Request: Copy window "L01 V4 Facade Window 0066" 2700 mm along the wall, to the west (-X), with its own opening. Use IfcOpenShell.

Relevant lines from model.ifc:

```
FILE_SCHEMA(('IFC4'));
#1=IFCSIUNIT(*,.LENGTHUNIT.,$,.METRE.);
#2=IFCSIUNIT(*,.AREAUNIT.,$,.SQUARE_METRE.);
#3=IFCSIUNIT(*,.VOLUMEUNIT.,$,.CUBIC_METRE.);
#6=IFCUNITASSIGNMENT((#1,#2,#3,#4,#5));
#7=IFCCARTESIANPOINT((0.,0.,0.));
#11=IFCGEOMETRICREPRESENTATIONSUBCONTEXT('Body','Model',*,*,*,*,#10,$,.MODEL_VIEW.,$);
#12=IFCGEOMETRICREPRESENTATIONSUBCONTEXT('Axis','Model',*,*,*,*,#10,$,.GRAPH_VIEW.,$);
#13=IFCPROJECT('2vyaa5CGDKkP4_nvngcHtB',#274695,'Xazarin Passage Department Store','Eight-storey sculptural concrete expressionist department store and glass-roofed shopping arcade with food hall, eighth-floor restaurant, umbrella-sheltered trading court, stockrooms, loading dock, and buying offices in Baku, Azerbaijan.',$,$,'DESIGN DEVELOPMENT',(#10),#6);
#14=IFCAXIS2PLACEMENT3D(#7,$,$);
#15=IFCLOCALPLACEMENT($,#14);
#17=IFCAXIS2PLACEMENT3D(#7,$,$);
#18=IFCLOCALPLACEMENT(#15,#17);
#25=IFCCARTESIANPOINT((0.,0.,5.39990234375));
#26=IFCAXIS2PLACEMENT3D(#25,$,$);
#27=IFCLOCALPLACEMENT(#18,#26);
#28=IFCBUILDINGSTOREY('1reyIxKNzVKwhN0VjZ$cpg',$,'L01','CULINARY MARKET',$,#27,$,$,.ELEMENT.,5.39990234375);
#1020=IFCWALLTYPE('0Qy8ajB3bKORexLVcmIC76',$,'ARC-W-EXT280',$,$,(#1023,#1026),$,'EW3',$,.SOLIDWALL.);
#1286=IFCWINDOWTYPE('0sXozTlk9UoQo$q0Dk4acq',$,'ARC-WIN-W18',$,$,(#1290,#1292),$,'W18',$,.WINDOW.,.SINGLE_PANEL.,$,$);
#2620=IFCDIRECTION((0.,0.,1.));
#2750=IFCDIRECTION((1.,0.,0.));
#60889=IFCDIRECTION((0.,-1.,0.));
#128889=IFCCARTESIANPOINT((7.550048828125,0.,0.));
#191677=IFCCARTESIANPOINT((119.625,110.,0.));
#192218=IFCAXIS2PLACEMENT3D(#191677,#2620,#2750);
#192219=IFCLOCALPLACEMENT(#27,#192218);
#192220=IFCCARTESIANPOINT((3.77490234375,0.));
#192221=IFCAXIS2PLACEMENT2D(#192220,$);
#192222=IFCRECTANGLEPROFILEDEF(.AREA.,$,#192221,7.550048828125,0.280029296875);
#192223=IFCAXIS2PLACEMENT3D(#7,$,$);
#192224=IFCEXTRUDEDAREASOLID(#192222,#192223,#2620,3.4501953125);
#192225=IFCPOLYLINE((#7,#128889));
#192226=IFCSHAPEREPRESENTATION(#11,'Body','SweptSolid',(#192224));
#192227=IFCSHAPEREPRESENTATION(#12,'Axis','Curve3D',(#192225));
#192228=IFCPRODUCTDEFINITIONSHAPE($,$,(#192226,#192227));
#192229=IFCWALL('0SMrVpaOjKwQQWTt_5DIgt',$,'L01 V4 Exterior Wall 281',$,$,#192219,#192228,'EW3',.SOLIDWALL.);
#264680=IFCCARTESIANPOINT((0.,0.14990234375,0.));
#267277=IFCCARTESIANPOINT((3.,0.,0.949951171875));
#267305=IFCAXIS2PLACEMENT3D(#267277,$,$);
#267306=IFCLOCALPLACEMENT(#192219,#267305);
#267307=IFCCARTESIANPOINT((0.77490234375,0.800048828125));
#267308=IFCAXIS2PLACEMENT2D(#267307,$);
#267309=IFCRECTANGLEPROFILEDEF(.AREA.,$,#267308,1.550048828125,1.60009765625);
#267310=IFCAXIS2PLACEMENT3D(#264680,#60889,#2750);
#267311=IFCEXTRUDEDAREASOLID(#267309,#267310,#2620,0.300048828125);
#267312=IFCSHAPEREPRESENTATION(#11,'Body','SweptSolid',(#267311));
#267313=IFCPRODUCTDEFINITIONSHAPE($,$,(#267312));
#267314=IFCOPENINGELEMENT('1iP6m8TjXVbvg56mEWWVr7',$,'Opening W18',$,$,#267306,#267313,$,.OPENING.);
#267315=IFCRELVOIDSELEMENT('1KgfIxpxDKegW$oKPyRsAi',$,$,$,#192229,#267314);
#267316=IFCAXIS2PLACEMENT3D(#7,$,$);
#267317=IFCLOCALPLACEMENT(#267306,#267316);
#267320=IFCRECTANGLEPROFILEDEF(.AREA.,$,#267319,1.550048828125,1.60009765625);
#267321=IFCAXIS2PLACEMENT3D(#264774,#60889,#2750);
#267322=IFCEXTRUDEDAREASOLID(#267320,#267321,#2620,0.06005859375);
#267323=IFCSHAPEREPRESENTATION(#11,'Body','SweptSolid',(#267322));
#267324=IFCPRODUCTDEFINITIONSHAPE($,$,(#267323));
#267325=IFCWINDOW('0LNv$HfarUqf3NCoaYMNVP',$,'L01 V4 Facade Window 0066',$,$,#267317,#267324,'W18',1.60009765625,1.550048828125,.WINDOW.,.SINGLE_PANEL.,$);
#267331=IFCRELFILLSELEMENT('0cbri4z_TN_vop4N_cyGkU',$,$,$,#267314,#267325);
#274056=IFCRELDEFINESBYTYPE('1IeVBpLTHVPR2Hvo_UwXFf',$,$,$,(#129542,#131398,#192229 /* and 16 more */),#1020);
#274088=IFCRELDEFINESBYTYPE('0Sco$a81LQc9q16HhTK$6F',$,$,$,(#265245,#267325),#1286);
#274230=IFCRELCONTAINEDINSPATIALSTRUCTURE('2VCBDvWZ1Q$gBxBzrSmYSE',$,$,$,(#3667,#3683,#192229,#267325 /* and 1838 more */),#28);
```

```python
import ifcopenshell
import ifcopenshell.api.feature
import ifcopenshell.api.geometry
import ifcopenshell.api.root
import ifcopenshell.geom
import ifcopenshell.util.element
import ifcopenshell.util.placement
import ifcopenshell.util.shape

model = ifcopenshell.open("model.ifc")
settings = ifcopenshell.geom.settings()


def volume(element):
    """Net volume in cubic metres, openings subtracted."""
    shape = ifcopenshell.geom.create_shape(settings, element)
    return ifcopenshell.util.shape.get_volume(shape.geometry)


window = model.by_id(267325)
opening = window.FillsVoids[0].RelatingOpeningElement
wall = opening.VoidsElements[0].RelatingBuildingElement
before = volume(wall)
shift = ifcopenshell.util.placement.get_local_placement(wall.ObjectPlacement)[:3, 0] * -2.7

# copy_class copies the void relationship, type, container and properties, but no geometry.
new_opening = ifcopenshell.api.root.copy_class(model, product=opening)
new_opening.Representation = ifcopenshell.util.element.copy_deep(
    model, opening.Representation, exclude=["IfcGeometricRepresentationContext", "IfcRepresentationMap"]
)
new_window = ifcopenshell.api.root.copy_class(model, product=window)
new_window.Representation = ifcopenshell.util.element.copy_deep(
    model, window.Representation, exclude=["IfcGeometricRepresentationContext", "IfcRepresentationMap"]
)
new_window.Tag = None
ifcopenshell.api.feature.add_filling(model, opening=new_opening, element=new_window)

for old, new in ((opening, new_opening), (window, new_window)):
    matrix = ifcopenshell.util.placement.get_local_placement(old.ObjectPlacement)
    matrix[:3, 3] += shift
    ifcopenshell.api.geometry.edit_object_placement(model, product=new, matrix=matrix, is_si=False)

after = volume(wall)

print(f"wall volume {before:.3f} -> {after:.3f} m3")

model.write("model-out.ifc")
```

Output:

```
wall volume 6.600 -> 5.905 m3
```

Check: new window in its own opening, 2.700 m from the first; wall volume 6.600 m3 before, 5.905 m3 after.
